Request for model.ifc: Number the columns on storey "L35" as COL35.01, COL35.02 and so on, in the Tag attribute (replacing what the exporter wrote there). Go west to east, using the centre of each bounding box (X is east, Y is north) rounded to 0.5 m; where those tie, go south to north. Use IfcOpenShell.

First a look at what the model holds.

```python
import ifcopenshell
import ifcopenshell.util.element
import ifcopenshell.util.placement

model = ifcopenshell.open("model.ifc")
print(model.schema)
storey = next(s for s in model.by_type("IfcBuildingStorey") if s.Name == "L35")
columns = [e for e in ifcopenshell.util.element.get_decomposition(storey) if e.is_a("IfcColumn")]
for e in sorted(columns, key=lambda e: e.id()):
    origin = ifcopenshell.util.placement.get_local_placement(e.ObjectPlacement)[:3, 3]
    print(e.id(), e.Tag, e.Name, origin.round(2) + 0.0, sep=" | ")
```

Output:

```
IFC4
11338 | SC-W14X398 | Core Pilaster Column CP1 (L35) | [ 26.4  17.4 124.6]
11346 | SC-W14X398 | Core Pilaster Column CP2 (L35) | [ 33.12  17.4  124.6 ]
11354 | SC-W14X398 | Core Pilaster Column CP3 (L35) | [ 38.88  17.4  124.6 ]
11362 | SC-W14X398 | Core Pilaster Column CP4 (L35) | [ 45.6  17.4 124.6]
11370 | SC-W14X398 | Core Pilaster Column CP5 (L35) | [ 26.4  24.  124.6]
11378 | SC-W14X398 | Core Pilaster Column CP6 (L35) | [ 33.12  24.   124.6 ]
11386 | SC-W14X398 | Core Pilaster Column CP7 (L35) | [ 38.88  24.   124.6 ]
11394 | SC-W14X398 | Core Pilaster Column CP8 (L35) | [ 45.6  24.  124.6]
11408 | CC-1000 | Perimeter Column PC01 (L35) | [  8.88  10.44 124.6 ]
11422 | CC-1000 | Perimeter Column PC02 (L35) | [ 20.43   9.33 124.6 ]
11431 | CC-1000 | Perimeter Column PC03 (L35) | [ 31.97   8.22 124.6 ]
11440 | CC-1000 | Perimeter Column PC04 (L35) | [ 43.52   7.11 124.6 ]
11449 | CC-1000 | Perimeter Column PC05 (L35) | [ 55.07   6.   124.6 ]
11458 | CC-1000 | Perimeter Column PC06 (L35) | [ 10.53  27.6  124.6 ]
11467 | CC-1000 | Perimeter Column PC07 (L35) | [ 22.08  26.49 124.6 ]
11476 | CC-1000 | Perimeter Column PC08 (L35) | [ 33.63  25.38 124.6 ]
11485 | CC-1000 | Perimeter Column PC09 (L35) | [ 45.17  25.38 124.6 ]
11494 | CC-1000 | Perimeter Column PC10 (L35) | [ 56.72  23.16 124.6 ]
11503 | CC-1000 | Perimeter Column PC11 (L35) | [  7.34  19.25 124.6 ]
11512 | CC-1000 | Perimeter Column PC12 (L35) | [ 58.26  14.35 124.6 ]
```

```python
import ifcopenshell
import ifcopenshell.geom
import ifcopenshell.util.element
import ifcopenshell.util.shape

model = ifcopenshell.open("model.ifc")
settings = ifcopenshell.geom.settings()
settings.set("use-world-coords", True)


def centre(element):
    shape = ifcopenshell.geom.create_shape(settings, element)
    return ifcopenshell.util.shape.get_bbox_centroid(shape.geometry)


storey = next(s for s in model.by_type("IfcBuildingStorey") if s.Name == "L35")
columns = [e for e in ifcopenshell.util.element.get_decomposition(storey) if e.is_a("IfcColumn")]

# Insertion points can sit at a corner or the storey origin, so sort by the geometry (in metres).
centres = {e: centre(e) for e in columns}
columns.sort(key=lambda e: (round(centres[e][0] / 0.5), centres[e][1]))

for i, e in enumerate(columns, start=1):
    number = f"COL35.{i:02d}"
    e.Tag = number
    print(e.id(), number)

model.write("model-out.ifc")
```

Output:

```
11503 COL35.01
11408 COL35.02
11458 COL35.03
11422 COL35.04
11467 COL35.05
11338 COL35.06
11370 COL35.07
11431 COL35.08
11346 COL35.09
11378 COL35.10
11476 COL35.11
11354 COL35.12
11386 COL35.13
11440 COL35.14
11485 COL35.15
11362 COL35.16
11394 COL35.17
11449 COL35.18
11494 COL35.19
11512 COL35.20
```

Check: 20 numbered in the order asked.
